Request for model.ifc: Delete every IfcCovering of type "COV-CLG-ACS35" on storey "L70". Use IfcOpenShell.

First a look at what the model holds.

```python
import ifcopenshell
import ifcopenshell.util.element

model = ifcopenshell.open("model.ifc")
print(model.schema)
storey = next(s for s in model.by_type("IfcBuildingStorey") if s.Name == "L70")
coverings = [e for e in ifcopenshell.util.element.get_decomposition(storey) if e.is_a("IfcCovering")]
seen = {}
for e in coverings:
    element_type = ifcopenshell.util.element.get_type(e)
    name = element_type.Name if element_type not in (None, e) else None
    seen[name] = seen.get(name, 0) + 1
for name, count in sorted(seen.items(), key=str):
    print(count, "x", name)
```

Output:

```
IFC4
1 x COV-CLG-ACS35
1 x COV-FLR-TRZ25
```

```python
import ifcopenshell
import ifcopenshell.api.root
import ifcopenshell.util.element

model = ifcopenshell.open("model.ifc")

storey = next(s for s in model.by_type("IfcBuildingStorey") if s.Name == "L70")
coverings = [e for e in ifcopenshell.util.element.get_decomposition(storey) if e.is_a("IfcCovering")]
targets = [e for e in coverings if (t := ifcopenshell.util.element.get_type(e)) not in (None, e) and t.Name == "COV-CLG-ACS35"]

for e in targets:
    ifcopenshell.api.root.remove_product(model, product=e)
print(len(targets), "removed")

model.write("model_v2.ifc")
```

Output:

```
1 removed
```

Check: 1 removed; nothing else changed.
